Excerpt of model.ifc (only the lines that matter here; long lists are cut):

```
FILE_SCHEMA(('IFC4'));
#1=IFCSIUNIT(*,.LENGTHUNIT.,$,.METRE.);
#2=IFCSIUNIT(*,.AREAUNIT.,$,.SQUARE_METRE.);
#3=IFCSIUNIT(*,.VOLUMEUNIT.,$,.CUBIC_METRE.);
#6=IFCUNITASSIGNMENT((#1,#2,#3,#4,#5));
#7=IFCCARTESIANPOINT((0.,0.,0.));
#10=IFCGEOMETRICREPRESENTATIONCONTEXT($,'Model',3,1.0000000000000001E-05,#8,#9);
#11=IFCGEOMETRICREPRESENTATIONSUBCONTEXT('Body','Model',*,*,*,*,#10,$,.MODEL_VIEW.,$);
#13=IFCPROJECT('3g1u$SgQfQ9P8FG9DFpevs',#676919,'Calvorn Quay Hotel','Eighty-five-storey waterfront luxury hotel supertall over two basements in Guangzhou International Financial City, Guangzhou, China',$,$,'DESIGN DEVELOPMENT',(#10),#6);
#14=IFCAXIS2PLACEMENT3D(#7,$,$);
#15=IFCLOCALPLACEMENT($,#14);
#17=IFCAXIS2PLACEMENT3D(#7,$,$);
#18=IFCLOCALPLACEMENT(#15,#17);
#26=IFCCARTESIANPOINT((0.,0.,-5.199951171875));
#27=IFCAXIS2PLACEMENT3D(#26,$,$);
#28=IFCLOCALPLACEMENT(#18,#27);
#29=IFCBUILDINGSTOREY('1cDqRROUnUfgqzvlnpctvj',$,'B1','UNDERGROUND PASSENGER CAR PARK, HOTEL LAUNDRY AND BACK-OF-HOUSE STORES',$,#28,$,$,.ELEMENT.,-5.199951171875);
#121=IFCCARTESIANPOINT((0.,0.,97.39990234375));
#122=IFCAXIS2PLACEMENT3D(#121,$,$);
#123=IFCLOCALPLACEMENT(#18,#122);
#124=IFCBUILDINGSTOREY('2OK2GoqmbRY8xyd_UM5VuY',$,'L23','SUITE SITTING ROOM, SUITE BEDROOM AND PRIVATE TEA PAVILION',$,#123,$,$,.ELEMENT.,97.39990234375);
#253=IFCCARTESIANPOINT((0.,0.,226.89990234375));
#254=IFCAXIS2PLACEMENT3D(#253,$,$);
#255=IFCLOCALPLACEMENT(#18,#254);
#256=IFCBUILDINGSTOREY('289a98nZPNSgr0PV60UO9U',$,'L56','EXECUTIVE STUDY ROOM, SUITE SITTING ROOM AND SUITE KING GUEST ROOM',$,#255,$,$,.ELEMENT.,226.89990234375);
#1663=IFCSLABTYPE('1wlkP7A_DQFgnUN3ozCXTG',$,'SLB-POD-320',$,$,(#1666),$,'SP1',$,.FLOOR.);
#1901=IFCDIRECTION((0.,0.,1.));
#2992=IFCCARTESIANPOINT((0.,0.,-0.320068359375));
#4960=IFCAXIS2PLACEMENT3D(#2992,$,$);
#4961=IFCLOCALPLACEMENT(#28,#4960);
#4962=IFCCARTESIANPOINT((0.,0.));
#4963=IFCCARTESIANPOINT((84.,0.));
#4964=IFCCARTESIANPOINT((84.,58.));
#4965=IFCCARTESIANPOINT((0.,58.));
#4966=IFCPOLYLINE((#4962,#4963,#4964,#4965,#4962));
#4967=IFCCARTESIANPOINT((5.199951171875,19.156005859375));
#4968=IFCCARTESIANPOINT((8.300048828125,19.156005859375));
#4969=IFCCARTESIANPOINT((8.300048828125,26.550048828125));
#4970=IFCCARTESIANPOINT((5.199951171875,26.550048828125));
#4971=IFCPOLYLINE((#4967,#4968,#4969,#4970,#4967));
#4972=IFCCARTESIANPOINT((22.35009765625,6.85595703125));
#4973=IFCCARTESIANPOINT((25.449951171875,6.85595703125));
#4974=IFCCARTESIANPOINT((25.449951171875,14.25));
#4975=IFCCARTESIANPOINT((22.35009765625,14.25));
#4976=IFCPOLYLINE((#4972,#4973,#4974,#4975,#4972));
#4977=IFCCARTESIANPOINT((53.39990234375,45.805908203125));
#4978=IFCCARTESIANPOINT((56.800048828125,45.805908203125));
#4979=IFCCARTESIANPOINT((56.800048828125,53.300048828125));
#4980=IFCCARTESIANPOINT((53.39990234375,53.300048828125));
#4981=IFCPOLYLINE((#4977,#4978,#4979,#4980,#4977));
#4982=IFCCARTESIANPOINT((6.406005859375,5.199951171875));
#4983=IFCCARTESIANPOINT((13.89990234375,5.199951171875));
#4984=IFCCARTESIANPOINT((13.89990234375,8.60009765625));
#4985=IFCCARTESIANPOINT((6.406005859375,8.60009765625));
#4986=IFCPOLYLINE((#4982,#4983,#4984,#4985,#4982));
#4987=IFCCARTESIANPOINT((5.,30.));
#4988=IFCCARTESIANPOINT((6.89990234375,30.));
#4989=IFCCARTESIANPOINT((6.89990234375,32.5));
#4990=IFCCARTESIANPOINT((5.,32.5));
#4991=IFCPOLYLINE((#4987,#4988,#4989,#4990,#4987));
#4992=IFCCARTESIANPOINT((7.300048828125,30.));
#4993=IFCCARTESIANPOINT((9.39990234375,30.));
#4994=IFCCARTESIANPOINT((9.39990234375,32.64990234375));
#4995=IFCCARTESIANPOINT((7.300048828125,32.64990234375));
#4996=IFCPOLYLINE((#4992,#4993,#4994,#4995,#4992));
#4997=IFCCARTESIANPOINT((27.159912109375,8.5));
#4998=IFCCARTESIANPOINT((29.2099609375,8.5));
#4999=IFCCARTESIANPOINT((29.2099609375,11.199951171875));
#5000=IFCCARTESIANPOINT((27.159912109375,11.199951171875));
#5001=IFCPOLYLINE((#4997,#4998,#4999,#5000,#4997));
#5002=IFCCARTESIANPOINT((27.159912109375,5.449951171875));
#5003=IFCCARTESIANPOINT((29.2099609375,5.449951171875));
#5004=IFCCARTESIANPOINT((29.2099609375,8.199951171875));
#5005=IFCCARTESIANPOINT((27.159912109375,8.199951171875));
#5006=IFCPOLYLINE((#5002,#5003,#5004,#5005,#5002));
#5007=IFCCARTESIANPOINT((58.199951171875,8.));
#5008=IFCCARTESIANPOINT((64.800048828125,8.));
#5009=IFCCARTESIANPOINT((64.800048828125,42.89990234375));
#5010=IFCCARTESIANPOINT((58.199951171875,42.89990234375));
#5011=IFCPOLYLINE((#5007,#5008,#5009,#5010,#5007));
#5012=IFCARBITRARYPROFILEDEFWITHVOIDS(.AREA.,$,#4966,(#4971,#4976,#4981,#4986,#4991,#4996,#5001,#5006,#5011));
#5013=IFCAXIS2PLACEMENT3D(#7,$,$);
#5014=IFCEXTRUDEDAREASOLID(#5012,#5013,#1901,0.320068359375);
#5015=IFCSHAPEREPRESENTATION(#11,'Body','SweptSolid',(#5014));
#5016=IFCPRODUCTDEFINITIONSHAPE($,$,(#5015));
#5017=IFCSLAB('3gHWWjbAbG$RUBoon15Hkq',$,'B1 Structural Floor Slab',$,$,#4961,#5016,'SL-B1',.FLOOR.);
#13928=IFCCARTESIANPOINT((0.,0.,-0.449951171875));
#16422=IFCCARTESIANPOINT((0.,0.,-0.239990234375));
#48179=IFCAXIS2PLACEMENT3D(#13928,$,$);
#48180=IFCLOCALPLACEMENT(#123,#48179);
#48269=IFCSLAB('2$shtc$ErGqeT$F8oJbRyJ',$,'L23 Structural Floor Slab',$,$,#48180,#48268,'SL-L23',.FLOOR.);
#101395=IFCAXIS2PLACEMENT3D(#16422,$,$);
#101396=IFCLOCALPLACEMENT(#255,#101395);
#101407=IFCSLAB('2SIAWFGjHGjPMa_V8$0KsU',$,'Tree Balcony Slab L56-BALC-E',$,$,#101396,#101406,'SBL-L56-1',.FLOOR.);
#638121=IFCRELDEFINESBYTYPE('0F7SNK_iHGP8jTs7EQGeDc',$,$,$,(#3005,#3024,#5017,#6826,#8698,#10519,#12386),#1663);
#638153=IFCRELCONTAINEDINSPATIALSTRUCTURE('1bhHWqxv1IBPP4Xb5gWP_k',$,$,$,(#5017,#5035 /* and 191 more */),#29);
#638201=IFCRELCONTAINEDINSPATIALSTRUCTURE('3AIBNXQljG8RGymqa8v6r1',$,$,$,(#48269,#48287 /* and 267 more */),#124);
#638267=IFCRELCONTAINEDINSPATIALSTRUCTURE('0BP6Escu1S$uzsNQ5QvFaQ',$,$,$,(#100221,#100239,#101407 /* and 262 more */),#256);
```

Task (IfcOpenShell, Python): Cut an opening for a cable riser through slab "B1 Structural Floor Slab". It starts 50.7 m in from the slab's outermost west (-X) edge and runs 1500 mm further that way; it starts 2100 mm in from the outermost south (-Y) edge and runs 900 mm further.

```python
import numpy as np
import ifcopenshell
import ifcopenshell.api.feature
import ifcopenshell.api.geometry
import ifcopenshell.api.root
import ifcopenshell.geom
import ifcopenshell.util.placement
import ifcopenshell.util.representation
import ifcopenshell.util.shape
import ifcopenshell.util.unit

model = ifcopenshell.open("model.ifc")
unit_scale = ifcopenshell.util.unit.calculate_unit_scale(model)
settings = ifcopenshell.geom.settings()


def volume(element):
    """Net volume in cubic metres, openings subtracted."""
    shape = ifcopenshell.geom.create_shape(settings, element)
    return ifcopenshell.util.shape.get_volume(shape.geometry)


slab = model.by_guid("3gHWWjbAbG$RUBoon15Hkq")
before = volume(slab)

# Extent in the slab's own axes, in metres. The edges named are its -X and -Y sides.
slab_shape = ifcopenshell.geom.create_shape(settings, slab)
vertices = ifcopenshell.util.shape.get_vertices(slab_shape.geometry)
x_min, y_min, bottom = vertices.min(axis=0)
top = vertices[:, 2].max()

opening = ifcopenshell.api.root.create_entity(model, ifc_class="IfcOpeningElement", name="Cable riser opening", predefined_type="OPENING")
context = ifcopenshell.util.representation.get_context(model, "Model", "Body", "MODEL_VIEW")
width, depth = 1.5, 0.9
outline = [(0.0, 0.0), (width, 0.0), (width, depth), (0.0, depth), (0.0, 0.0)]
# Overshoot both faces by 50 mm so the cut is clean.
shape = ifcopenshell.api.geometry.add_slab_representation(
    model, context=context, depth=top - bottom + 0.1, polyline=outline
)
ifcopenshell.api.geometry.assign_representation(model, product=opening, representation=shape)

matrix = ifcopenshell.util.placement.get_local_placement(slab.ObjectPlacement)
matrix[:, 3] = matrix @ np.append(np.array([x_min + 50.7, y_min + 2.1, bottom - 0.05]) / unit_scale, 1.0)
ifcopenshell.api.geometry.edit_object_placement(model, product=opening, matrix=matrix, is_si=False)
ifcopenshell.api.feature.add_feature(model, feature=opening, element=slab)

after = volume(slab)

print(f"slab volume {before:.3f} -> {after:.3f} m3")

model.write("model_updated.ifc")
```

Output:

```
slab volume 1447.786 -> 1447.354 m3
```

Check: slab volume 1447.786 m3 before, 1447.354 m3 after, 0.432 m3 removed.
